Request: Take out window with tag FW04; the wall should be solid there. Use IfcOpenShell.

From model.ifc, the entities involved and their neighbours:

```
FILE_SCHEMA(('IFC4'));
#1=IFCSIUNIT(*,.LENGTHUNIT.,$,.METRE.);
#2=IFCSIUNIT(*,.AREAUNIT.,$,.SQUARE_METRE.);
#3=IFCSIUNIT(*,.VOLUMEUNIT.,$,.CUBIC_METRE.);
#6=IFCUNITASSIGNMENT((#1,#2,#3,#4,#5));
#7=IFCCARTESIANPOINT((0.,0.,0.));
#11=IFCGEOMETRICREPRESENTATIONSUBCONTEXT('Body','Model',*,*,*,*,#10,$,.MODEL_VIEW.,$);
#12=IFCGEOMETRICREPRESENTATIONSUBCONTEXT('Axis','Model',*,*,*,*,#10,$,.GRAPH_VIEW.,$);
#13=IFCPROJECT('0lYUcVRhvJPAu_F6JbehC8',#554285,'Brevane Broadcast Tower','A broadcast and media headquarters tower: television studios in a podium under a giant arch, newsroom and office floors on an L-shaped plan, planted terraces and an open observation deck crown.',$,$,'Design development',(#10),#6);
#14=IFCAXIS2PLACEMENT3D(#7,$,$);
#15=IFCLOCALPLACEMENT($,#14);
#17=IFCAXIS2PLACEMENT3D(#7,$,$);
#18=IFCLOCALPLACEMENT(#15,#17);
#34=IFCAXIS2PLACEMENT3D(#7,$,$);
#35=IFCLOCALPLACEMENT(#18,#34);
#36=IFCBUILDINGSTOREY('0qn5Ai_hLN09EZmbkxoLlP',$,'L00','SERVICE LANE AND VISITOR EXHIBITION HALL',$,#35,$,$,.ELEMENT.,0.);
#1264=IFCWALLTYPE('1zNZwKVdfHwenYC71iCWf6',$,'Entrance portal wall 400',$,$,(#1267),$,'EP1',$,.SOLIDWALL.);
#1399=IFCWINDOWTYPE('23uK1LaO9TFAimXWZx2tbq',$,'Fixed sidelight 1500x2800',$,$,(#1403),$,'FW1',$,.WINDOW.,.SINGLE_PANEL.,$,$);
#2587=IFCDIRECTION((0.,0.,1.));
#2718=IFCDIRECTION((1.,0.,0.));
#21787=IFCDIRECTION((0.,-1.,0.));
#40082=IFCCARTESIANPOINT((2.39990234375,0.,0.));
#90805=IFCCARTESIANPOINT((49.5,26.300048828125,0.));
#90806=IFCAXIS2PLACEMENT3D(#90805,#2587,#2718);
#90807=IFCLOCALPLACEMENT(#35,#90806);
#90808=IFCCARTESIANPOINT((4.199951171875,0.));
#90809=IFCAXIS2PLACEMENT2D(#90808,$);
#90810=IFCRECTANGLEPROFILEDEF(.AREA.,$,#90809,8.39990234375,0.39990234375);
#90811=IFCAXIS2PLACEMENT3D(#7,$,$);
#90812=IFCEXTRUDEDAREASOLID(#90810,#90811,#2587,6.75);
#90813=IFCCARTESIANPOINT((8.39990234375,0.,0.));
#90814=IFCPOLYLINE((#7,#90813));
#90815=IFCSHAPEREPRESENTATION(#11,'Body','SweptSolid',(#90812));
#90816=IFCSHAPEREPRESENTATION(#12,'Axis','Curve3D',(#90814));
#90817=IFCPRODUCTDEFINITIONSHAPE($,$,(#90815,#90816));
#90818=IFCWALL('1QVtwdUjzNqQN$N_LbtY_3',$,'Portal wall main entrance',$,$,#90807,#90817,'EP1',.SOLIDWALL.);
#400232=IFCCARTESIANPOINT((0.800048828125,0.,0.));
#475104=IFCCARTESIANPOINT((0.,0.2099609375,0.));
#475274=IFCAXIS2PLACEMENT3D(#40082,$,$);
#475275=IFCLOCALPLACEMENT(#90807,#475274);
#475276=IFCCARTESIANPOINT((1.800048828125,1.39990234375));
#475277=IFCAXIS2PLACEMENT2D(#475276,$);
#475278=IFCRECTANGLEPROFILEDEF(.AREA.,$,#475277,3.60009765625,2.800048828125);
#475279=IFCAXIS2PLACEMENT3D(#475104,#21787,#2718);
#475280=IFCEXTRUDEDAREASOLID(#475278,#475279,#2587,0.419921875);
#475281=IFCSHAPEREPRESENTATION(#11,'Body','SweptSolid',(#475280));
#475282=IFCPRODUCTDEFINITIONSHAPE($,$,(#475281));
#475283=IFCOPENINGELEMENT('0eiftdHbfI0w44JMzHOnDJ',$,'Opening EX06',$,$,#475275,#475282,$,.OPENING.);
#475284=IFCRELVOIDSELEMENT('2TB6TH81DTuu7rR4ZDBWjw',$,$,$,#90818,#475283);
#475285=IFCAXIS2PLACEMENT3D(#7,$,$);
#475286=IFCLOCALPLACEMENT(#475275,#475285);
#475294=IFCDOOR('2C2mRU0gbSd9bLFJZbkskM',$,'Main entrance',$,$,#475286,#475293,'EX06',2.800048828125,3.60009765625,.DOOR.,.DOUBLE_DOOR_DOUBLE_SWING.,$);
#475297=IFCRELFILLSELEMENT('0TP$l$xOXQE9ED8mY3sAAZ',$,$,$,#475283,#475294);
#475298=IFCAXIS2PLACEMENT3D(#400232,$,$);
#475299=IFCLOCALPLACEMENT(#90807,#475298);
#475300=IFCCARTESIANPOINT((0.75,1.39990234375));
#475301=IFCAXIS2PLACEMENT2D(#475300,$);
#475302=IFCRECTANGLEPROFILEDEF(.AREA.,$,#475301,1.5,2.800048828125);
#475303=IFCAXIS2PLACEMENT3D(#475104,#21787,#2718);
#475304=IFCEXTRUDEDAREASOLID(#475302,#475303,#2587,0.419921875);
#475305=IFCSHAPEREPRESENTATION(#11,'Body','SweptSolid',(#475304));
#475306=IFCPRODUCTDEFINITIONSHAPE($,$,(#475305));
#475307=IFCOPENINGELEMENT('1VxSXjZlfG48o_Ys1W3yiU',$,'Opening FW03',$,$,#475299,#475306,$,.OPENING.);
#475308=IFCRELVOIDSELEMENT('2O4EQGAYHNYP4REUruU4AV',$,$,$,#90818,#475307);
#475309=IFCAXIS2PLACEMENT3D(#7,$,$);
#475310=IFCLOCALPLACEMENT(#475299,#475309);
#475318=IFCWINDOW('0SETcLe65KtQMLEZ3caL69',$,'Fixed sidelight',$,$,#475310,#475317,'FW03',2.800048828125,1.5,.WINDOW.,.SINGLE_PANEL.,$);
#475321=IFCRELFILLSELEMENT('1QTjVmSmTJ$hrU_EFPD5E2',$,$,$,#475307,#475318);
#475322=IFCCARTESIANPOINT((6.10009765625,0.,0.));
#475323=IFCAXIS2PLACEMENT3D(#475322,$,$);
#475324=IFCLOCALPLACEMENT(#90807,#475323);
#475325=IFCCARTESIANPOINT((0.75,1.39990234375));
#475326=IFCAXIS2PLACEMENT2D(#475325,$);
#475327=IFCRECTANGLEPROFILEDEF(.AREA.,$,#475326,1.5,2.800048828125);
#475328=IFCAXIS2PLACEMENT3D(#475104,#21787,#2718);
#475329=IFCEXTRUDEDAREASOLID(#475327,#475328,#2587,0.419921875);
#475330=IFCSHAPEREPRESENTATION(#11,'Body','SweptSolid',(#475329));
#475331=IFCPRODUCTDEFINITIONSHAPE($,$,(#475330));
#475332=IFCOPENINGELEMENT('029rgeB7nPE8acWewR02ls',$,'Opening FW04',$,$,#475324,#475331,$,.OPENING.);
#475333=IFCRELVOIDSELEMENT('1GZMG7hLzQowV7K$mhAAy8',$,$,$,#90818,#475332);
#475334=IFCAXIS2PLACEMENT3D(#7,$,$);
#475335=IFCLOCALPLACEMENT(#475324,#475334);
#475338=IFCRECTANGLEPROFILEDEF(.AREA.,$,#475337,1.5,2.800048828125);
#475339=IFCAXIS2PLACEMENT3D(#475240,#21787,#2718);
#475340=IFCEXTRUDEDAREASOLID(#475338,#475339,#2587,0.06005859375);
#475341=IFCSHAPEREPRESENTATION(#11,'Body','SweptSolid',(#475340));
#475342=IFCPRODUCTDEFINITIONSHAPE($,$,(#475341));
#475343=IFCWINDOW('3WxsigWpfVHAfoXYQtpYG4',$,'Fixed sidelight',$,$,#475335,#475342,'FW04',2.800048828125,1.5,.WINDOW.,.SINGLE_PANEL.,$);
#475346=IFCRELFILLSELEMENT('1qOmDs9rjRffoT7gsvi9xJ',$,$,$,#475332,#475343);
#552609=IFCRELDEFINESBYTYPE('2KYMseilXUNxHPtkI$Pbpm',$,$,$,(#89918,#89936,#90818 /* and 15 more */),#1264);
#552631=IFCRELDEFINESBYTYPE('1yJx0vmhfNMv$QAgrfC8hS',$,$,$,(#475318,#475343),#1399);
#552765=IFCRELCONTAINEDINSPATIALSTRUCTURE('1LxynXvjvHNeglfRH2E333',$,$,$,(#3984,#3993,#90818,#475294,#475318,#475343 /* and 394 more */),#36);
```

```python
import ifcopenshell
import ifcopenshell.api.feature
import ifcopenshell.api.root
import ifcopenshell.geom
import ifcopenshell.util.shape

model = ifcopenshell.open("model.ifc")
settings = ifcopenshell.geom.settings()


def volume(element):
    """Net volume in cubic metres, openings subtracted."""
    shape = ifcopenshell.geom.create_shape(settings, element)
    return ifcopenshell.util.shape.get_volume(shape.geometry)


window = model.by_id(475343)
opening = window.FillsVoids[0].RelatingOpeningElement
wall = opening.VoidsElements[0].RelatingBuildingElement
before = volume(wall)

ifcopenshell.api.root.remove_product(model, product=window)
ifcopenshell.api.feature.remove_feature(model, feature=opening)

after = volume(wall)

print(f"wall volume {before:.3f} -> {after:.3f} m3")

model.write("model_edited.ifc")
```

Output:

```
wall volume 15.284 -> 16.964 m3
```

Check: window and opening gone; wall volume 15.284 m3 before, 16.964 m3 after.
